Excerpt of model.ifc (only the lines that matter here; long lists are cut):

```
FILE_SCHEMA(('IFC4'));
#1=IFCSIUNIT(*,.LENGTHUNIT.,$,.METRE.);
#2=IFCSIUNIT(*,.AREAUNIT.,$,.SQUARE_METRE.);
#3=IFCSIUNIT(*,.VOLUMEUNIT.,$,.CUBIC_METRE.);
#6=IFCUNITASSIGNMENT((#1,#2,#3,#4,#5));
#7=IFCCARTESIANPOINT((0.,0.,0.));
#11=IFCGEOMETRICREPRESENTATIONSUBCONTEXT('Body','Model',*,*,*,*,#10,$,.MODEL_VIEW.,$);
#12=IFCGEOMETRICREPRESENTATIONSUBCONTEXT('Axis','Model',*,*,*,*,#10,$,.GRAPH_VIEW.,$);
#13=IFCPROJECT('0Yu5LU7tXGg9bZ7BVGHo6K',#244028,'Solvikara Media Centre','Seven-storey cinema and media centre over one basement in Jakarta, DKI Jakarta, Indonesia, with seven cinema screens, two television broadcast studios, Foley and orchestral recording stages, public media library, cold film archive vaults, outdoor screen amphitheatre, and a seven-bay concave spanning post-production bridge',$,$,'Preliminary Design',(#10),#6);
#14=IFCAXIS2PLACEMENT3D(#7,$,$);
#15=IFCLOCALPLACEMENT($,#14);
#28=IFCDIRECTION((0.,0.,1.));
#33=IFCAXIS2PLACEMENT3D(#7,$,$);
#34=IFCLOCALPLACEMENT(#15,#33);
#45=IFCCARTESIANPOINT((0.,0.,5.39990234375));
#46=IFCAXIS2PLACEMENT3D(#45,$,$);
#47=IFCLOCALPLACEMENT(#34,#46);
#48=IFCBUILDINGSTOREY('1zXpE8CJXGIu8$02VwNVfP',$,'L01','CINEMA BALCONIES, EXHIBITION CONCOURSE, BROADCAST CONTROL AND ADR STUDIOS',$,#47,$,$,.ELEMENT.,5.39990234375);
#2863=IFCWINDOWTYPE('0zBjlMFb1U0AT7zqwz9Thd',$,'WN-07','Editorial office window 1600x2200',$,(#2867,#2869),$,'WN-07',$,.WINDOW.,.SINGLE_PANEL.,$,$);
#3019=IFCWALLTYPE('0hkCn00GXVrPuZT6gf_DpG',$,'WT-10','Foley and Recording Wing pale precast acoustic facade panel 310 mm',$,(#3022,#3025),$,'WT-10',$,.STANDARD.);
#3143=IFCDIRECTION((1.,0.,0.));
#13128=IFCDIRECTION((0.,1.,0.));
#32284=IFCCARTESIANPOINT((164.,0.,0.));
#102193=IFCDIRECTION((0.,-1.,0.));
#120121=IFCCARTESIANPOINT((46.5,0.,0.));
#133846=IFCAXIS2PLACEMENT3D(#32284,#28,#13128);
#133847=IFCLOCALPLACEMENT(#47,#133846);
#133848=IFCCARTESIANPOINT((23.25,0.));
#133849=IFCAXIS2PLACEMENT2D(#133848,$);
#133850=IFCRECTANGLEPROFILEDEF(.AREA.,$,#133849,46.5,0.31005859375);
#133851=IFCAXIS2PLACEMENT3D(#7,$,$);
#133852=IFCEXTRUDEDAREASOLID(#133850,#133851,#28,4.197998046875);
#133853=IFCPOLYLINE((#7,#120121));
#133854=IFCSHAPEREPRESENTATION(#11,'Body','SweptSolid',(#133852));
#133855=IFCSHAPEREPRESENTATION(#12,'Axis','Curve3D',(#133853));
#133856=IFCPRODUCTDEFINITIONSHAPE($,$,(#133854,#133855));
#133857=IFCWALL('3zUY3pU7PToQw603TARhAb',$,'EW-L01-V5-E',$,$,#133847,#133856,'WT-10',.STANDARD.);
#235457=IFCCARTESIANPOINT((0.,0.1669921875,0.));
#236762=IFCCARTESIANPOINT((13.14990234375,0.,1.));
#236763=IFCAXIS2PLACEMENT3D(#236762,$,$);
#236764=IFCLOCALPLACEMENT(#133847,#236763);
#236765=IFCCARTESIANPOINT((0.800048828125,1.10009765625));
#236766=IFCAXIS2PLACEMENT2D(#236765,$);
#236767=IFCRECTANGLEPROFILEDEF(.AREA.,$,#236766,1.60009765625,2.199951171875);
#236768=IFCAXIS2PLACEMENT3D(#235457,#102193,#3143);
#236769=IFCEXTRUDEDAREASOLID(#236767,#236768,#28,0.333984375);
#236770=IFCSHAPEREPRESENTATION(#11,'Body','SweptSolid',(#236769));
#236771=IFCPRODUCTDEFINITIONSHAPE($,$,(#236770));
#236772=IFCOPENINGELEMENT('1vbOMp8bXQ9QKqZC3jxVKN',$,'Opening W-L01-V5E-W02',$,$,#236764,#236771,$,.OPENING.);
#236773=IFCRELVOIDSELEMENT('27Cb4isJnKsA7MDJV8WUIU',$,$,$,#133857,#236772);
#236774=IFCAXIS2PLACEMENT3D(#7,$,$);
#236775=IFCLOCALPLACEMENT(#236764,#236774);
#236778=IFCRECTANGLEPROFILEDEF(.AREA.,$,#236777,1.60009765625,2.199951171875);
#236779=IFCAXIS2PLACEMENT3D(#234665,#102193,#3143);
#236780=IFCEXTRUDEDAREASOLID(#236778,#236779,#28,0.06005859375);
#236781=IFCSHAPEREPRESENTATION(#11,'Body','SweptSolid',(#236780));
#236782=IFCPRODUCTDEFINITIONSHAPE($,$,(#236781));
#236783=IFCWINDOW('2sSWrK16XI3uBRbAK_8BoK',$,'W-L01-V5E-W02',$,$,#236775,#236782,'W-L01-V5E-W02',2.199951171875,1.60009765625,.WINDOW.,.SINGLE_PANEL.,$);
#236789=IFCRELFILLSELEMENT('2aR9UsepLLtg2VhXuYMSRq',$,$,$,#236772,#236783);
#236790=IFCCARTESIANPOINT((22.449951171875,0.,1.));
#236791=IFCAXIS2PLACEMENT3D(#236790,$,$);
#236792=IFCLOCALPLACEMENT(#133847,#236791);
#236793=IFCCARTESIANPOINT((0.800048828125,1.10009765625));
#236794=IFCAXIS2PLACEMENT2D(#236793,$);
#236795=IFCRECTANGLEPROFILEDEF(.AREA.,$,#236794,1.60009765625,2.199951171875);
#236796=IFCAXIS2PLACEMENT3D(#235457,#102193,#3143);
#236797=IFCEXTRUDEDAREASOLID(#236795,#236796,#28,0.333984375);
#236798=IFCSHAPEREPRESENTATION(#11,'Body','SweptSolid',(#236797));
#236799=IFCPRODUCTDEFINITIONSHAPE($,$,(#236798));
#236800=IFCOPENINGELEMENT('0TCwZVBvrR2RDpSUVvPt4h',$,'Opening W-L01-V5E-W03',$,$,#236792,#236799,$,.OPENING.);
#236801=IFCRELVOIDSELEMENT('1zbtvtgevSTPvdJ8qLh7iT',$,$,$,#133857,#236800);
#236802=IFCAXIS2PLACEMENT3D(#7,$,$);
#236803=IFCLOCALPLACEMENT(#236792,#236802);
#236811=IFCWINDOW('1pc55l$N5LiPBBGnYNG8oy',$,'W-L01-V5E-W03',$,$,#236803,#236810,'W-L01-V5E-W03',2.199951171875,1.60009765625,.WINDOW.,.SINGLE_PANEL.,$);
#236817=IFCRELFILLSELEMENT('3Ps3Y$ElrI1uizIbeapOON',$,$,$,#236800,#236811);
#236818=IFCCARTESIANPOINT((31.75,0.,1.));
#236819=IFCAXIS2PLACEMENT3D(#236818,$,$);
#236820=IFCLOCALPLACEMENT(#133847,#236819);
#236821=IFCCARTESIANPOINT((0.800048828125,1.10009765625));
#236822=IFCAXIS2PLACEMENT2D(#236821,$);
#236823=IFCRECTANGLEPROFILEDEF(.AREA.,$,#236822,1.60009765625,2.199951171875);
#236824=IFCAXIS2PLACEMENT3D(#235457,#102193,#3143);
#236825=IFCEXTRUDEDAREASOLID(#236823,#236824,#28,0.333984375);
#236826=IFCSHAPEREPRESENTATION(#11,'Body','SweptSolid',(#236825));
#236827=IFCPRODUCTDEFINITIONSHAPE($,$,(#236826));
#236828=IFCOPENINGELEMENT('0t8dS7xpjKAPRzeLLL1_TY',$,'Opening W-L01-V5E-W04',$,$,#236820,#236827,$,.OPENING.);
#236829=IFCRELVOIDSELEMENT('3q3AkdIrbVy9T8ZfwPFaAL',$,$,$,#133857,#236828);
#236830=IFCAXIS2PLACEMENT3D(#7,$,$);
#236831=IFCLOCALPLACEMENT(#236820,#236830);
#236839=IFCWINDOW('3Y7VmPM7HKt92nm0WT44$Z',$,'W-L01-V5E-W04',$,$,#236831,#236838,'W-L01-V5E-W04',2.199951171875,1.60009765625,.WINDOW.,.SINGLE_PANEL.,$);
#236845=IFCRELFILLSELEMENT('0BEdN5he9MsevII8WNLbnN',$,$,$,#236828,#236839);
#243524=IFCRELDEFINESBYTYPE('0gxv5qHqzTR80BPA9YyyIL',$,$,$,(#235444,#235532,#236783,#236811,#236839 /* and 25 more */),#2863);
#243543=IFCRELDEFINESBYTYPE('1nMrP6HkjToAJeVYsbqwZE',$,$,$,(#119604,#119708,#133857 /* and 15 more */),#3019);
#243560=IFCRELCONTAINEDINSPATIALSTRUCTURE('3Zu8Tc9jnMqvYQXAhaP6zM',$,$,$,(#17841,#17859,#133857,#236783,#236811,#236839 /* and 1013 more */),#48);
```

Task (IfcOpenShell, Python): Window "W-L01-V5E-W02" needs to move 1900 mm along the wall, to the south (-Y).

```python
import ifcopenshell
import ifcopenshell.api.geometry
import ifcopenshell.util.placement

model = ifcopenshell.open("model.ifc")

window = model.by_guid("2sSWrK16XI3uBRbAK_8BoK")
opening = window.FillsVoids[0].RelatingOpeningElement
wall = opening.VoidsElements[0].RelatingBuildingElement

wall_matrix = ifcopenshell.util.placement.get_local_placement(wall.ObjectPlacement)
shift = wall_matrix[:3, 0] * -1.9
before = ifcopenshell.util.placement.get_local_placement(window.ObjectPlacement)[:3, 3].copy()

# The window is placed relative to its opening, so it follows when the opening moves.
matrix = ifcopenshell.util.placement.get_local_placement(opening.ObjectPlacement)
matrix[:3, 3] += shift
ifcopenshell.api.geometry.edit_object_placement(
    model, product=opening, matrix=matrix, is_si=False, should_transform_children=True
)

after = ifcopenshell.util.placement.get_local_placement(window.ObjectPlacement)[:3, 3]
print("window moved by", (after - before).round(3) + 0.0)

model.write("model_edited.ifc")
```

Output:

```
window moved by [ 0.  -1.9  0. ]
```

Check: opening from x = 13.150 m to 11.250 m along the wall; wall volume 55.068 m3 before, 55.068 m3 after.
